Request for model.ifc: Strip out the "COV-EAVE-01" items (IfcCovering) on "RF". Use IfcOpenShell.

First a look at what the model holds.

```python
import ifcopenshell
import ifcopenshell.util.element

model = ifcopenshell.open("model.ifc")
print(model.schema)
storey = next(s for s in model.by_type("IfcBuildingStorey") if s.Name == "RF")
coverings = [e for e in ifcopenshell.util.element.get_decomposition(storey) if e.is_a("IfcCovering")]
seen = {}
for e in coverings:
    element_type = ifcopenshell.util.element.get_type(e)
    name = element_type.Name if element_type not in (None, e) else None
    seen[name] = seen.get(name, 0) + 1
for name, count in sorted(seen.items(), key=str):
    print(count, "x", name)
```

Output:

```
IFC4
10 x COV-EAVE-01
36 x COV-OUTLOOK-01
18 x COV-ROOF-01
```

```python
import ifcopenshell
import ifcopenshell.api.root
import ifcopenshell.util.element

model = ifcopenshell.open("model.ifc")

storey = next(s for s in model.by_type("IfcBuildingStorey") if s.Name == "RF")
coverings = [e for e in ifcopenshell.util.element.get_decomposition(storey) if e.is_a("IfcCovering")]
targets = [e for e in coverings if (t := ifcopenshell.util.element.get_type(e)) not in (None, e) and t.Name == "COV-EAVE-01"]

for e in targets:
    ifcopenshell.api.root.remove_product(model, product=e)
print(len(targets), "removed")

model.write("model_v2.ifc")
```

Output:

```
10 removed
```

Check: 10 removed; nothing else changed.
